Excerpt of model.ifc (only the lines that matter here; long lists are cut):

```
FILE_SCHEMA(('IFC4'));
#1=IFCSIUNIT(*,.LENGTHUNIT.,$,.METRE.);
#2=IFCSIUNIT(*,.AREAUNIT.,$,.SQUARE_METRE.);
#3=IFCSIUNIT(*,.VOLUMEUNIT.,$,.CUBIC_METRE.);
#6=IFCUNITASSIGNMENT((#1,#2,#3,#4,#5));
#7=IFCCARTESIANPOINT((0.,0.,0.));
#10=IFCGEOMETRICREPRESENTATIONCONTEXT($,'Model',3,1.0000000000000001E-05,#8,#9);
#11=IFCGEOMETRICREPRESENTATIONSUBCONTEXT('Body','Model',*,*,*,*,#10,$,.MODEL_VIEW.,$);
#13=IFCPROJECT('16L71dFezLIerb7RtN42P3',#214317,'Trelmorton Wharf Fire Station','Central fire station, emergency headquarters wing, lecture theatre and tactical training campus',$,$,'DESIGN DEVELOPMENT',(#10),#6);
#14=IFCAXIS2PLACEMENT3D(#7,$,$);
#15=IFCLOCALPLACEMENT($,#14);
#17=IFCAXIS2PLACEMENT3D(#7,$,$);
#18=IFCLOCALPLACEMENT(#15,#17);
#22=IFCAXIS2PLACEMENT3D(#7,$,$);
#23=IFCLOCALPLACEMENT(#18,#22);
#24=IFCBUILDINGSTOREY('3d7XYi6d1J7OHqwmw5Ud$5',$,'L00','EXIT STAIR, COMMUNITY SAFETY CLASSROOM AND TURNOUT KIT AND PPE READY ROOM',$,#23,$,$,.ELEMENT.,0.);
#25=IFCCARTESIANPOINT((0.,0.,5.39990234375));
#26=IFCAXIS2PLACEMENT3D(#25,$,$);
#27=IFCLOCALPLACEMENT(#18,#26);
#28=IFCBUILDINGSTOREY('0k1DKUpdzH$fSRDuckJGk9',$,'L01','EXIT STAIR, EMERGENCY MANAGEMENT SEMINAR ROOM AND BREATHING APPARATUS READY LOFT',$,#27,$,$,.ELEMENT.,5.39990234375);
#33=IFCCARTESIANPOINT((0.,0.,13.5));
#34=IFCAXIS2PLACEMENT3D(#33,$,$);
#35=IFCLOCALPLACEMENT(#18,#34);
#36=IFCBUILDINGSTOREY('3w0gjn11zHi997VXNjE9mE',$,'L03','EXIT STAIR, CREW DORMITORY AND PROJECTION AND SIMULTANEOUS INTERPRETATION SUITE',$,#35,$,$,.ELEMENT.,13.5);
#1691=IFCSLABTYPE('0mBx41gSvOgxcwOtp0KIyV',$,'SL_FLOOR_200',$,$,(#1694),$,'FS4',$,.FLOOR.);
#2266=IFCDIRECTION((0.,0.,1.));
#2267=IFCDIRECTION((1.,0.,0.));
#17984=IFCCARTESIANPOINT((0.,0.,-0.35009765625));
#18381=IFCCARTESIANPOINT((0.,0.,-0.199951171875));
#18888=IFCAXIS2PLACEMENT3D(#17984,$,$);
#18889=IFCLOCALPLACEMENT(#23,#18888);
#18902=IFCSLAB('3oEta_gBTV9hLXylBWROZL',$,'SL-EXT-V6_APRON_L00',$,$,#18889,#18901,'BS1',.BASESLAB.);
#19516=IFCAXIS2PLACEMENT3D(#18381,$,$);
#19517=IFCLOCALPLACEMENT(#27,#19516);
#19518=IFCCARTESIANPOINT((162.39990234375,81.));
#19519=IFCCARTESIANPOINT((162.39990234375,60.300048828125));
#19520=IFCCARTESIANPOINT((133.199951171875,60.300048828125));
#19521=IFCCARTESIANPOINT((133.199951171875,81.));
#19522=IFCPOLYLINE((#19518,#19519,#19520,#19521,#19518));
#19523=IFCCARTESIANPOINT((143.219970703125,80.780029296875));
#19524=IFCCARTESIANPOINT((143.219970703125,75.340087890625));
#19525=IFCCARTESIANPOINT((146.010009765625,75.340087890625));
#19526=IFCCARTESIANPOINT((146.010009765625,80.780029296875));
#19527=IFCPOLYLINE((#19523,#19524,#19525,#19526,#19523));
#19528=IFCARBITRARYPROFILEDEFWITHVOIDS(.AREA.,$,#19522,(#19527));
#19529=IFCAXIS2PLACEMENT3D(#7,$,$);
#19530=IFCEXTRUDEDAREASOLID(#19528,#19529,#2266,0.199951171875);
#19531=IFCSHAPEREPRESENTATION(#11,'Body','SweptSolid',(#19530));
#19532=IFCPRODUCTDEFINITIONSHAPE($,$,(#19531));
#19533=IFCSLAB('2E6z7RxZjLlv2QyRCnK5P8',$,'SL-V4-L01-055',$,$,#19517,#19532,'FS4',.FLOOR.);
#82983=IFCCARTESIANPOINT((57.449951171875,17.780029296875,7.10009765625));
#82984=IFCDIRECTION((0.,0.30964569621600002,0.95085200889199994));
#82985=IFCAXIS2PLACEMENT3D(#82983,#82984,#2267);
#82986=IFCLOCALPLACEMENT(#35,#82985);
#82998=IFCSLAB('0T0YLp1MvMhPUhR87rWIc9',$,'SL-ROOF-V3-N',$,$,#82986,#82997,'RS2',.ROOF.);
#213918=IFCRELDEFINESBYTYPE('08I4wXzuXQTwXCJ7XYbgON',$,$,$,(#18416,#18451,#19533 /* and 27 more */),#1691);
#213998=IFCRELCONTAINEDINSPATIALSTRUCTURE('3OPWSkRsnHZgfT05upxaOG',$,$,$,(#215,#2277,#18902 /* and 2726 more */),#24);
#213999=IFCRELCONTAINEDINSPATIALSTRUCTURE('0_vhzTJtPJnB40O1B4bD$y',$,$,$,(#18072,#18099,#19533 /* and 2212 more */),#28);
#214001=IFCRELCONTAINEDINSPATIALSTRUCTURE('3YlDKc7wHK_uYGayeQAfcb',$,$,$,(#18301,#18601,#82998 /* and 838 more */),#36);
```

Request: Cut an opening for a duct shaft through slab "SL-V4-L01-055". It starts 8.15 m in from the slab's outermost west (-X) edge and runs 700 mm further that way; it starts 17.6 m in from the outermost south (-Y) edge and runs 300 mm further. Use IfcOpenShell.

```python
import numpy as np
import ifcopenshell
import ifcopenshell.api.feature
import ifcopenshell.api.geometry
import ifcopenshell.api.root
import ifcopenshell.geom
import ifcopenshell.util.placement
import ifcopenshell.util.representation
import ifcopenshell.util.shape
import ifcopenshell.util.unit

model = ifcopenshell.open("model.ifc")
unit_scale = ifcopenshell.util.unit.calculate_unit_scale(model)
settings = ifcopenshell.geom.settings()


def volume(element):
    """Net volume in cubic metres, openings subtracted."""
    shape = ifcopenshell.geom.create_shape(settings, element)
    return ifcopenshell.util.shape.get_volume(shape.geometry)


slab = model.by_guid("2E6z7RxZjLlv2QyRCnK5P8")
before = volume(slab)

# Extent in the slab's own axes, in metres. The edges named are its -X and -Y sides.
slab_shape = ifcopenshell.geom.create_shape(settings, slab)
vertices = ifcopenshell.util.shape.get_vertices(slab_shape.geometry)
x_min, y_min, bottom = vertices.min(axis=0)
top = vertices[:, 2].max()

opening = ifcopenshell.api.root.create_entity(model, ifc_class="IfcOpeningElement", name="Duct shaft opening", predefined_type="OPENING")
context = ifcopenshell.util.representation.get_context(model, "Model", "Body", "MODEL_VIEW")
width, depth = 0.7, 0.3
outline = [(0.0, 0.0), (width, 0.0), (width, depth), (0.0, depth), (0.0, 0.0)]
# Overshoot both faces by 50 mm so the cut is clean.
shape = ifcopenshell.api.geometry.add_slab_representation(
    model, context=context, depth=top - bottom + 0.1, polyline=outline
)
ifcopenshell.api.geometry.assign_representation(model, product=opening, representation=shape)

matrix = ifcopenshell.util.placement.get_local_placement(slab.ObjectPlacement)
matrix[:, 3] = matrix @ np.append(np.array([x_min + 8.15, y_min + 17.6, bottom - 0.05]) / unit_scale, 1.0)
ifcopenshell.api.geometry.edit_object_placement(model, product=opening, matrix=matrix, is_si=False)
ifcopenshell.api.feature.add_feature(model, feature=opening, element=slab)

after = volume(slab)

print(f"slab volume {before:.3f} -> {after:.3f} m3")

model.write("model_rev.ifc")
```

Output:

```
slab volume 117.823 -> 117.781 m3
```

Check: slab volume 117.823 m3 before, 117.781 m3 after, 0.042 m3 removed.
